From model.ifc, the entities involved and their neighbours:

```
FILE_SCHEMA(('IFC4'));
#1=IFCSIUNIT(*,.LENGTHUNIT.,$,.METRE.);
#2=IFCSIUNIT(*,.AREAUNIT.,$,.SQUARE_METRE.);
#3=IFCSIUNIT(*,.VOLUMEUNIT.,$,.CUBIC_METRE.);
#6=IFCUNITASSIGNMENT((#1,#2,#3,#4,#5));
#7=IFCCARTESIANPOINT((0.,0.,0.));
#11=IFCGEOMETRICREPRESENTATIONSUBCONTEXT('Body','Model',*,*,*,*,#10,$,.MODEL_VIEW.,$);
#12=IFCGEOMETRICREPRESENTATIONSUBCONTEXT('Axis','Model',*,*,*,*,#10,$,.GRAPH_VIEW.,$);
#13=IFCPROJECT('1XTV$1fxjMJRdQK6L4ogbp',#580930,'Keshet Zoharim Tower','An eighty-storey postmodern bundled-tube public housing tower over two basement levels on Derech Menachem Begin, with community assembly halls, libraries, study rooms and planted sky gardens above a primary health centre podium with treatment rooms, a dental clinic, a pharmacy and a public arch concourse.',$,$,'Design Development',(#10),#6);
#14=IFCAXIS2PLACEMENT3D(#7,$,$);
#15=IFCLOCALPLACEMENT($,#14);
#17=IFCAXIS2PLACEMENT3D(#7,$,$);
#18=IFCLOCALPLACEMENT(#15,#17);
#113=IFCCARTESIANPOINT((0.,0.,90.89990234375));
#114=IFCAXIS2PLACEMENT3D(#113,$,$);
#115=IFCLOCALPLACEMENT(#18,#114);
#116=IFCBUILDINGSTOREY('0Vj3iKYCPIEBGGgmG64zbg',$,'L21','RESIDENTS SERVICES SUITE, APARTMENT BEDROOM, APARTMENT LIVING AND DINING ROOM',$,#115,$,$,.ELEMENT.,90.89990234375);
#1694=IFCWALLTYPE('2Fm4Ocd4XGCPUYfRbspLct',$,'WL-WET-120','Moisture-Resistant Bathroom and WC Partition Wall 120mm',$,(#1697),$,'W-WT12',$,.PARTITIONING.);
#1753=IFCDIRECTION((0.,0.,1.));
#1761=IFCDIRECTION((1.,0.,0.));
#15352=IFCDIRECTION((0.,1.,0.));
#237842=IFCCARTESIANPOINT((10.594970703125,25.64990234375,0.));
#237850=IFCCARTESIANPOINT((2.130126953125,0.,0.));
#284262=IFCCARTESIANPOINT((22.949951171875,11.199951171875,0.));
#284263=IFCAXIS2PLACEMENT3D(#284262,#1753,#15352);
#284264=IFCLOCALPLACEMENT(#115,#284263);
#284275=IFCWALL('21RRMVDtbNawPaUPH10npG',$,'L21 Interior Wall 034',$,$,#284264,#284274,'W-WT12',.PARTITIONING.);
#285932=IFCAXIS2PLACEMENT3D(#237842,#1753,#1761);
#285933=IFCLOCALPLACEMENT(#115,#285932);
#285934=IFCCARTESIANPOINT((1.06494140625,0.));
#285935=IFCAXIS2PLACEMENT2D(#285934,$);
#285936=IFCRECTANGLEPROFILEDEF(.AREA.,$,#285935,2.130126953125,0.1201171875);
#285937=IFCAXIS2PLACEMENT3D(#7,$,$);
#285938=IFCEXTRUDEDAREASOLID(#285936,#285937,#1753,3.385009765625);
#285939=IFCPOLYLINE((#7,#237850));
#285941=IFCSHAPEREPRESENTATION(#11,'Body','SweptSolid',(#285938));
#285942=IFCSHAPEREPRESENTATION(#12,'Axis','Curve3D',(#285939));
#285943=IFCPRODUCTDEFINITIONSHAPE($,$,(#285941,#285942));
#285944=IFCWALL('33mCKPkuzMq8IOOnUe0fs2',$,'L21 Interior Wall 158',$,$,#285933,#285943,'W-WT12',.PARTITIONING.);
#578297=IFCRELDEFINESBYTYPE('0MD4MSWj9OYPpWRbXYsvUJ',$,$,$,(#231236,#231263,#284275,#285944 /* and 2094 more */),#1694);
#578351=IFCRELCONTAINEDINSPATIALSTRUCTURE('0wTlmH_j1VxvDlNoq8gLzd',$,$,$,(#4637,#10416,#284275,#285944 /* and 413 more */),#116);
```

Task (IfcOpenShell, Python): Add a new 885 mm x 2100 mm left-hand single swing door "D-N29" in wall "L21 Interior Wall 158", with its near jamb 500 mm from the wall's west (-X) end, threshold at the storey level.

```python
import numpy as np
import ifcopenshell
import ifcopenshell.api.feature
import ifcopenshell.api.geometry
import ifcopenshell.api.root
import ifcopenshell.api.spatial
import ifcopenshell.geom
import ifcopenshell.util.element
import ifcopenshell.util.placement
import ifcopenshell.util.representation
import ifcopenshell.util.shape
import ifcopenshell.util.unit

model = ifcopenshell.open("model.ifc")
unit_scale = ifcopenshell.util.unit.calculate_unit_scale(model)
settings = ifcopenshell.geom.settings()


def volume(element):
    """Net volume in cubic metres, openings subtracted."""
    shape = ifcopenshell.geom.create_shape(settings, element)
    return ifcopenshell.util.shape.get_volume(shape.geometry)


wall = model.by_guid("33mCKPkuzMq8IOOnUe0fs2")
storey = ifcopenshell.util.element.get_container(wall, ifc_class="IfcBuildingStorey")
context = ifcopenshell.util.representation.get_context(model, "Model", "Body", "MODEL_VIEW")
before = volume(wall)

width, height, from_end, sill = 0.885, 2.1, 0.5, 0.0  # metres

# The wall runs along its own X axis, and the end named is its -X end.
wall_shape = ifcopenshell.geom.create_shape(settings, wall)
x, y, z = ifcopenshell.util.shape.get_vertices(wall_shape.geometry).T
start = x.min() + from_end
face, thickness = float(y.min()), float(y.max() - y.min())
wall_matrix = ifcopenshell.util.placement.get_local_placement(wall.ObjectPlacement)
level = ifcopenshell.util.placement.get_local_placement(storey.ObjectPlacement)[2, 3]


def in_wall(x, y):
    """Placement at x, y metres in the wall's axes, at sill height."""
    matrix = wall_matrix.copy()
    matrix[:, 3] = wall_matrix @ np.array([x / unit_scale, y / unit_scale, 0.0, 1.0])
    matrix[2, 3] = level + sill / unit_scale
    return matrix


# Opening: a box that overshoots both wall faces by 50 mm.
opening = ifcopenshell.api.root.create_entity(model, ifc_class="IfcOpeningElement", predefined_type="OPENING")
box = ifcopenshell.api.geometry.add_wall_representation(
    model, context=context, length=width, height=height, thickness=thickness + 0.1
)
ifcopenshell.api.geometry.assign_representation(model, product=opening, representation=box)
ifcopenshell.api.geometry.edit_object_placement(model, product=opening, matrix=in_wall(start, face - 0.05), is_si=False)
ifcopenshell.api.feature.add_feature(model, feature=opening, element=wall)

door = ifcopenshell.api.root.create_entity(model, ifc_class="IfcDoor", name="D-N29", predefined_type="DOOR")
door.OverallWidth, door.OverallHeight = width / unit_scale, height / unit_scale
door.OperationType = "SINGLE_SWING_LEFT"
body = ifcopenshell.api.geometry.add_door_representation(
    model,
    context=context,
    overall_width=door.OverallWidth,
    overall_height=door.OverallHeight,
    operation_type="SINGLE_SWING_LEFT",
    lining_properties={"LiningDepth": thickness / unit_scale, "ThresholdDepth": thickness / unit_scale},
)
ifcopenshell.api.geometry.assign_representation(model, product=door, representation=body)
ifcopenshell.api.spatial.assign_container(model, products=[door], relating_structure=storey)
ifcopenshell.api.feature.add_filling(model, opening=opening, element=door)

# The lining spans the wall, so the door starts at the wall face.
ifcopenshell.api.geometry.edit_object_placement(model, product=door, matrix=in_wall(start, face), is_si=False)

after = volume(wall)

print(f"wall volume {before:.3f} -> {after:.3f} m3")

model.write("model_edited.ifc")
```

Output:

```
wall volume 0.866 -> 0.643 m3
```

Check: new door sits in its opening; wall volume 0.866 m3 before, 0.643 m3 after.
